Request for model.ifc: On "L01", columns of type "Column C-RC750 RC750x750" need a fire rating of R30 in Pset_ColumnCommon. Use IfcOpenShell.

First a look at what the model holds.

```python
import ifcopenshell
import ifcopenshell.util.element

model = ifcopenshell.open("model.ifc")
print(model.schema)
storey = next(s for s in model.by_type("IfcBuildingStorey") if s.Name == "L01")
columns = [e for e in ifcopenshell.util.element.get_decomposition(storey) if e.is_a("IfcColumn")]
seen = {}
for e in columns:
    element_type = ifcopenshell.util.element.get_type(e)
    key = (element_type.Name if element_type != e and element_type else None, ifcopenshell.util.element.get_pset(e, "Pset_ColumnCommon", "FireRating"))
    seen[key] = seen.get(key, 0) + 1
for (name, value), count in sorted(seen.items(), key=str):
    print(count, "x", name, "|", value)
```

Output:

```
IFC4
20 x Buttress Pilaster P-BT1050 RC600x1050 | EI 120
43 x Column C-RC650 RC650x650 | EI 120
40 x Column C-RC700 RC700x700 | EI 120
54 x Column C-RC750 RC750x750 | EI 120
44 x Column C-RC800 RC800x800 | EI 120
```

```python
import ifcopenshell
import ifcopenshell.api.pset
import ifcopenshell.util.element

model = ifcopenshell.open("model.ifc")

storey = next(s for s in model.by_type("IfcBuildingStorey") if s.Name == "L01")
columns = [e for e in ifcopenshell.util.element.get_decomposition(storey) if e.is_a("IfcColumn")]

count = 0
for e in columns:
    element_type = ifcopenshell.util.element.get_type(e)
    if element_type in (None, e) or element_type.Name != "Column C-RC750 RC750x750":
        continue
    # add_pset returns the element's existing set when there is one.
    pset = ifcopenshell.api.pset.add_pset(model, product=e, name="Pset_ColumnCommon")
    ifcopenshell.api.pset.edit_pset(model, pset=pset, properties={"FireRating": "R30"})
    count += 1

print(count, "columns updated")

model.write("model-out.ifc")
```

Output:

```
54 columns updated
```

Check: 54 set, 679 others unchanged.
